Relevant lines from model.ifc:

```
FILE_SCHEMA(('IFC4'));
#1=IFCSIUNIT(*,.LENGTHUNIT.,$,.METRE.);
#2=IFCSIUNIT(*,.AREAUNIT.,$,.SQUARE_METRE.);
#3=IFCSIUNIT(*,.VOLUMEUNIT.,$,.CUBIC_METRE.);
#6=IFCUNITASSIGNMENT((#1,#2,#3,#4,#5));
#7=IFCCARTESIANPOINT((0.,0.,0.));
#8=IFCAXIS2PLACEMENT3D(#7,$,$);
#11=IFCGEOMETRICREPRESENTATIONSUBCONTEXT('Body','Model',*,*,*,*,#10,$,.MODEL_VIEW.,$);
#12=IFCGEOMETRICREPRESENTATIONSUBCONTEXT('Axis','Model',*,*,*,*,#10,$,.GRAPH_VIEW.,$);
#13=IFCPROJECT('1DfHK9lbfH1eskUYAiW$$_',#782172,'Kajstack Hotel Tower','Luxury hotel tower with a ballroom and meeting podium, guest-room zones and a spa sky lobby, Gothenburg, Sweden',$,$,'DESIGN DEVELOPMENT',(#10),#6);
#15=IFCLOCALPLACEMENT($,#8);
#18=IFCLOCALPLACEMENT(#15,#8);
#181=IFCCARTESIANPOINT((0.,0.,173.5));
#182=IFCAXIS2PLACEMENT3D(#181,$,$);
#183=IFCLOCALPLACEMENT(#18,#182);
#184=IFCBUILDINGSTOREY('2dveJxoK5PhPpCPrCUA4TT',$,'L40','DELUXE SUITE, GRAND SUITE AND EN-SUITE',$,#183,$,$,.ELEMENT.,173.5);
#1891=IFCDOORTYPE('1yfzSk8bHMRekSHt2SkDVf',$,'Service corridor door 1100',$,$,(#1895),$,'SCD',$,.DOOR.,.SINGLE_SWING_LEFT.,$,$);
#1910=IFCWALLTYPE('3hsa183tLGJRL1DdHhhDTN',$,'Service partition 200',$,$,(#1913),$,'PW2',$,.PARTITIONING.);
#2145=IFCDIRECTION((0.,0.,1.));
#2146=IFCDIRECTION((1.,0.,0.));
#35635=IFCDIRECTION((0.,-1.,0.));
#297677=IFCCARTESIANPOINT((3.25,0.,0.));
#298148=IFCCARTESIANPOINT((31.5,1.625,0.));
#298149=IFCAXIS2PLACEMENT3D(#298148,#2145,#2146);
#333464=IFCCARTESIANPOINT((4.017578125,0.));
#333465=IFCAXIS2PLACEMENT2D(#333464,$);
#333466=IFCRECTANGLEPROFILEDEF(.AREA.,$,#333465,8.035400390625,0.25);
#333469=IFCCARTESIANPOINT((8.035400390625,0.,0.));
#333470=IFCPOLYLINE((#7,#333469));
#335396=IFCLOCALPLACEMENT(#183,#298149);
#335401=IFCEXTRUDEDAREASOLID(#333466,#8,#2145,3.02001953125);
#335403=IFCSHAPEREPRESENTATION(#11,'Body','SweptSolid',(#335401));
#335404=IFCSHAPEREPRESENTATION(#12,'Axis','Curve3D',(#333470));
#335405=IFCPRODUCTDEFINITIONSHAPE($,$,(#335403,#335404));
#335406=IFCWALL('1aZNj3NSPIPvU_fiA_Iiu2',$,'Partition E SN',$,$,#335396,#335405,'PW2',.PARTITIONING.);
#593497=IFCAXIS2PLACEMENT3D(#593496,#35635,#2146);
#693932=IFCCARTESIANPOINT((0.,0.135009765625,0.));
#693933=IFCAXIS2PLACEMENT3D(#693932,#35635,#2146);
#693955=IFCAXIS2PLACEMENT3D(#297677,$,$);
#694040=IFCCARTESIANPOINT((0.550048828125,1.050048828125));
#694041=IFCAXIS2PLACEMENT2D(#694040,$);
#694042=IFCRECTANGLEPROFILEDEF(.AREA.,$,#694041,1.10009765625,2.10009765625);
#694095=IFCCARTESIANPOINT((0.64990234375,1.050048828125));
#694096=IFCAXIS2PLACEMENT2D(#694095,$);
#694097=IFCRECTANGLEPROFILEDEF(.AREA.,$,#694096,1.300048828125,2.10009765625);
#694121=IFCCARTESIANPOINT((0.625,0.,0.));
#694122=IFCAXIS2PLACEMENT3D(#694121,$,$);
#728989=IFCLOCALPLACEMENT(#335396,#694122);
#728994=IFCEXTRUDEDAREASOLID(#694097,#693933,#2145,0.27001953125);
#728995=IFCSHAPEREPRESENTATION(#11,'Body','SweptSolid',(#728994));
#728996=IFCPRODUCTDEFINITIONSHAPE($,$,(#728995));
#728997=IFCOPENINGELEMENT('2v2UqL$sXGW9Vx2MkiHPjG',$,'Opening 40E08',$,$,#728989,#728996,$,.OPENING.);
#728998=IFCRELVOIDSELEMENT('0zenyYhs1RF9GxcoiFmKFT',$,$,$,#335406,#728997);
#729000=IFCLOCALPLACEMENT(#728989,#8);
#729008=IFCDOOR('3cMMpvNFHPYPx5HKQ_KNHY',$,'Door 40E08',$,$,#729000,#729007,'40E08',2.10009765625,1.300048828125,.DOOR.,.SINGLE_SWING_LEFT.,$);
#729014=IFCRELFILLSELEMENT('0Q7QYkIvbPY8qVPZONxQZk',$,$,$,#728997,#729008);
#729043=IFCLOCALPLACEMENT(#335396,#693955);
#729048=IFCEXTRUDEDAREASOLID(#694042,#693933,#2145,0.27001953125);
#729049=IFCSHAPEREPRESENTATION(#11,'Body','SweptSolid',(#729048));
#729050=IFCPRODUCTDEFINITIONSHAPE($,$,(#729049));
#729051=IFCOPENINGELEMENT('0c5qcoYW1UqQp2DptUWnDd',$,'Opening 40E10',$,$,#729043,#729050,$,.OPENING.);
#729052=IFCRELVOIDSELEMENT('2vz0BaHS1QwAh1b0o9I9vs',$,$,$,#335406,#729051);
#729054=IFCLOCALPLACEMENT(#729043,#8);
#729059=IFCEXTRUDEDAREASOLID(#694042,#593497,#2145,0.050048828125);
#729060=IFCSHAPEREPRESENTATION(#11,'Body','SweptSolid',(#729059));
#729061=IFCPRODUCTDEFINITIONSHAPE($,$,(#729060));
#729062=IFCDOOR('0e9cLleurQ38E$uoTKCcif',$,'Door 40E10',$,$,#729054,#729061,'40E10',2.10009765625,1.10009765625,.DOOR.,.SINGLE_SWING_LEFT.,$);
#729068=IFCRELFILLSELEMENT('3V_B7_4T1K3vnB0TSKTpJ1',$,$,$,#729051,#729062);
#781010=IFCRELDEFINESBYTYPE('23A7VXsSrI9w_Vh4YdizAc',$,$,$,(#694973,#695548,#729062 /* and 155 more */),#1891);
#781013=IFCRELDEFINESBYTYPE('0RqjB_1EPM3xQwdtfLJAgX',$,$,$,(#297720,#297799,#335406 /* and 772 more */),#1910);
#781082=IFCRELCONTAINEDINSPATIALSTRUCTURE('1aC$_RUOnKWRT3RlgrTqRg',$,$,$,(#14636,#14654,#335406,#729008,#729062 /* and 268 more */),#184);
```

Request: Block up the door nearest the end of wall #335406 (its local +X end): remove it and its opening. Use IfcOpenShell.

```python
import ifcopenshell
import ifcopenshell.api.feature
import ifcopenshell.api.root
import ifcopenshell.geom
import ifcopenshell.util.shape

model = ifcopenshell.open("model.ifc")
settings = ifcopenshell.geom.settings()


def volume(element):
    """Net volume in cubic metres, openings subtracted."""
    shape = ifcopenshell.geom.create_shape(settings, element)
    return ifcopenshell.util.shape.get_volume(shape.geometry)


door = model.by_guid("0e9cLleurQ38E$uoTKCcif")
opening = door.FillsVoids[0].RelatingOpeningElement
wall = opening.VoidsElements[0].RelatingBuildingElement
before = volume(wall)

ifcopenshell.api.root.remove_product(model, product=door)
ifcopenshell.api.feature.remove_feature(model, feature=opening)

after = volume(wall)

print(f"wall volume {before:.3f} -> {after:.3f} m3")

model.write("model_edited.ifc")
```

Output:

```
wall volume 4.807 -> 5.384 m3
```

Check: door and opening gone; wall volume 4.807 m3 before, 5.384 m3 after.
